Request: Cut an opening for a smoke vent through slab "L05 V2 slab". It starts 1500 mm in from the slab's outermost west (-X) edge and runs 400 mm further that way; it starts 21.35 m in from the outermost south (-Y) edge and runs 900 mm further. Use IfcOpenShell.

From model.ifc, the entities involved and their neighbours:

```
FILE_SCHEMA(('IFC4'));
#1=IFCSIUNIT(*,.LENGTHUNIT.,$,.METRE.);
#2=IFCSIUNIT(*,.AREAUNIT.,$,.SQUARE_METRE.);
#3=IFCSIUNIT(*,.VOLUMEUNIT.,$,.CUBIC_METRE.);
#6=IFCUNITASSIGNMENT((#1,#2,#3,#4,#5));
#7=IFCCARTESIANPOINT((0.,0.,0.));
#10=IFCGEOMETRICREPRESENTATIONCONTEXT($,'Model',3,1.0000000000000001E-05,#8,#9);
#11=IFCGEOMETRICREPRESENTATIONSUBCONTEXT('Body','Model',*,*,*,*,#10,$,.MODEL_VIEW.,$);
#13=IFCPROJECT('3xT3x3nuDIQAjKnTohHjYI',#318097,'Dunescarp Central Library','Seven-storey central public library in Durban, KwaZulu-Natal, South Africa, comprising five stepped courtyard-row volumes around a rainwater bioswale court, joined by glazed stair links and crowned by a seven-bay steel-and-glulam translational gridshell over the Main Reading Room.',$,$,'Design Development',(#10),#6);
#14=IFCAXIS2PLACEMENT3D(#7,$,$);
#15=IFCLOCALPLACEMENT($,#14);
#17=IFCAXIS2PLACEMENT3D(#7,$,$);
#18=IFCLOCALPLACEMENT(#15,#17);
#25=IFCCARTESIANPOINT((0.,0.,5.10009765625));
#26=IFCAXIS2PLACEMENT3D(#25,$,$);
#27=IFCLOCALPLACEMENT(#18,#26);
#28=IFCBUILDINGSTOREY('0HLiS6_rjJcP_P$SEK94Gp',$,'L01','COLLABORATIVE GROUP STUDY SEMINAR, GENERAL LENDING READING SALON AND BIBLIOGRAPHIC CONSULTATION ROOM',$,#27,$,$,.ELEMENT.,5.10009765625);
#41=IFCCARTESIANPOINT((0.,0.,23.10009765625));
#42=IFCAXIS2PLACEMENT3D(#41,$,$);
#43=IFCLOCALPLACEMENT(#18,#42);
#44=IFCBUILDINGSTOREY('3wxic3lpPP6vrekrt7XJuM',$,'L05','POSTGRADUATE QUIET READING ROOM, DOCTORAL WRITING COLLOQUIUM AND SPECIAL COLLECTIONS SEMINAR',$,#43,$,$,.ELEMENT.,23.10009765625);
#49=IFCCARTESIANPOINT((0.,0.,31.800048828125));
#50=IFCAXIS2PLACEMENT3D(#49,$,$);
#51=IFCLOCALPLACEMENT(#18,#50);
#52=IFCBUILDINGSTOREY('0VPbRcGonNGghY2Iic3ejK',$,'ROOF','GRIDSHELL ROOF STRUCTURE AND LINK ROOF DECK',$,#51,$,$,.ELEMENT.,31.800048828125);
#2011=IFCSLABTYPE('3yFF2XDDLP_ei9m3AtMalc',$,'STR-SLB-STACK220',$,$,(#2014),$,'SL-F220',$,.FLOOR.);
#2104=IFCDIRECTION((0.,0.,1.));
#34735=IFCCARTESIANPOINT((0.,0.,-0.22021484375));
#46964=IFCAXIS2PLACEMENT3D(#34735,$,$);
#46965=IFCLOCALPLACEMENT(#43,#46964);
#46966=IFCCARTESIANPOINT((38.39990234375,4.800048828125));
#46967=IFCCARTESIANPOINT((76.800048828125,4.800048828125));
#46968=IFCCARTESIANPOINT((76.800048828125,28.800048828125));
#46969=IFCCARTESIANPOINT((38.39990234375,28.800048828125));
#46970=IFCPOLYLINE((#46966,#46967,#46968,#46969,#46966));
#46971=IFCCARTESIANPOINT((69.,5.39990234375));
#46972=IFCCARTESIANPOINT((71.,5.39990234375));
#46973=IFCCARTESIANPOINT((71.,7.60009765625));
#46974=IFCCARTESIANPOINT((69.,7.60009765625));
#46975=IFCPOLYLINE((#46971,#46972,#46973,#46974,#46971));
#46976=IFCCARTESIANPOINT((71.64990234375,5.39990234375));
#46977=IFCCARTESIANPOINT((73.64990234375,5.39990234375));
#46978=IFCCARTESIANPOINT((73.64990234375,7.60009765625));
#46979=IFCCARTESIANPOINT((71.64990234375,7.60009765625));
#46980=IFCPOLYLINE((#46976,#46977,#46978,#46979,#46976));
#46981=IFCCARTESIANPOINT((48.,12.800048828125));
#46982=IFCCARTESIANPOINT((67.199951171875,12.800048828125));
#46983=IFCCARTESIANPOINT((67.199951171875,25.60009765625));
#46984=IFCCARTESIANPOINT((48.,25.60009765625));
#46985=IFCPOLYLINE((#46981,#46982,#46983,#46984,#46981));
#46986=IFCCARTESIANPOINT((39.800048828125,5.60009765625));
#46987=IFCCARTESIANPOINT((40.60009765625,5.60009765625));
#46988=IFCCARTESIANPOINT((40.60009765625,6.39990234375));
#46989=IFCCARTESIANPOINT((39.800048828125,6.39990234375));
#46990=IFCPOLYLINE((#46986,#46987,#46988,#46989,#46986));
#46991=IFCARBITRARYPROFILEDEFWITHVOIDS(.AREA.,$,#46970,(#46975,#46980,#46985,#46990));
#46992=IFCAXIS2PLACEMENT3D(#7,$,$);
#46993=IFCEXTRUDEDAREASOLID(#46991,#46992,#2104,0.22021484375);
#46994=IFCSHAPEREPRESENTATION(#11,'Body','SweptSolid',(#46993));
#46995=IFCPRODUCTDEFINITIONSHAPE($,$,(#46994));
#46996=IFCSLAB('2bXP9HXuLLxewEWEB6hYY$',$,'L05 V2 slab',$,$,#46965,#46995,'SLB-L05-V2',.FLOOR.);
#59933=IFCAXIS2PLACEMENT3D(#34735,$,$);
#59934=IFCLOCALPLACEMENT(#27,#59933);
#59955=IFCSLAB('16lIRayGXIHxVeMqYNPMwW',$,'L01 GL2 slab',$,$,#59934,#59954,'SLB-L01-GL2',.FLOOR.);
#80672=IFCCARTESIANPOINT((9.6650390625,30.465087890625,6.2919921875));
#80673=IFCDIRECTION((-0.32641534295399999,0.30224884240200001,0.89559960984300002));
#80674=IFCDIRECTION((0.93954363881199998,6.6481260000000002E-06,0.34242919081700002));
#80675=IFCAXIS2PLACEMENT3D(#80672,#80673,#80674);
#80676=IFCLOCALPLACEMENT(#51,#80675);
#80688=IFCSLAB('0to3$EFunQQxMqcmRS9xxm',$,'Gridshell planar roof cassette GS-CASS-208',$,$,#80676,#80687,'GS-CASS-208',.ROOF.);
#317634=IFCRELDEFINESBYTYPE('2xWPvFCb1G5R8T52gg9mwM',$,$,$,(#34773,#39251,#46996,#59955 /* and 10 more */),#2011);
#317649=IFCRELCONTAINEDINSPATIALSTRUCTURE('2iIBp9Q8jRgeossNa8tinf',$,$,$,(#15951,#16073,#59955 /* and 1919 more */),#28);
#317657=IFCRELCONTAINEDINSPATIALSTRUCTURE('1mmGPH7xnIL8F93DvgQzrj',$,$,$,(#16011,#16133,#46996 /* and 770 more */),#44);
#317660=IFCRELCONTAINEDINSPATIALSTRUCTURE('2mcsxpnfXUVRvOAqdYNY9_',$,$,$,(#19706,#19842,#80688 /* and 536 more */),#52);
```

```python
import numpy as np
import ifcopenshell
import ifcopenshell.api.feature
import ifcopenshell.api.geometry
import ifcopenshell.api.root
import ifcopenshell.geom
import ifcopenshell.util.placement
import ifcopenshell.util.representation
import ifcopenshell.util.shape
import ifcopenshell.util.unit

model = ifcopenshell.open("model.ifc")
unit_scale = ifcopenshell.util.unit.calculate_unit_scale(model)
settings = ifcopenshell.geom.settings()


def volume(element):
    """Net volume in cubic metres, openings subtracted."""
    shape = ifcopenshell.geom.create_shape(settings, element)
    return ifcopenshell.util.shape.get_volume(shape.geometry)


slab = model.by_id(46996)
before = volume(slab)

# Extent in the slab's own axes, in metres. The edges named are its -X and -Y sides.
slab_shape = ifcopenshell.geom.create_shape(settings, slab)
vertices = ifcopenshell.util.shape.get_vertices(slab_shape.geometry)
x_min, y_min, bottom = vertices.min(axis=0)
top = vertices[:, 2].max()

opening = ifcopenshell.api.root.create_entity(model, ifc_class="IfcOpeningElement", name="Smoke vent opening", predefined_type="OPENING")
context = ifcopenshell.util.representation.get_context(model, "Model", "Body", "MODEL_VIEW")
width, depth = 0.4, 0.9
outline = [(0.0, 0.0), (width, 0.0), (width, depth), (0.0, depth), (0.0, 0.0)]
# Overshoot both faces by 50 mm so the cut is clean.
shape = ifcopenshell.api.geometry.add_slab_representation(
    model, context=context, depth=top - bottom + 0.1, polyline=outline
)
ifcopenshell.api.geometry.assign_representation(model, product=opening, representation=shape)

matrix = ifcopenshell.util.placement.get_local_placement(slab.ObjectPlacement)
matrix[:, 3] = matrix @ np.append(np.array([x_min + 1.5, y_min + 21.35, bottom - 0.05]) / unit_scale, 1.0)
ifcopenshell.api.geometry.edit_object_placement(model, product=opening, matrix=matrix, is_si=False)
ifcopenshell.api.feature.add_feature(model, feature=opening, element=slab)

after = volume(slab)

print(f"slab volume {before:.3f} -> {after:.3f} m3")

model.write("model-out.ifc")
```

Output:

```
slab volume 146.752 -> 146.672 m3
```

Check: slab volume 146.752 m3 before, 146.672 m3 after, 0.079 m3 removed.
